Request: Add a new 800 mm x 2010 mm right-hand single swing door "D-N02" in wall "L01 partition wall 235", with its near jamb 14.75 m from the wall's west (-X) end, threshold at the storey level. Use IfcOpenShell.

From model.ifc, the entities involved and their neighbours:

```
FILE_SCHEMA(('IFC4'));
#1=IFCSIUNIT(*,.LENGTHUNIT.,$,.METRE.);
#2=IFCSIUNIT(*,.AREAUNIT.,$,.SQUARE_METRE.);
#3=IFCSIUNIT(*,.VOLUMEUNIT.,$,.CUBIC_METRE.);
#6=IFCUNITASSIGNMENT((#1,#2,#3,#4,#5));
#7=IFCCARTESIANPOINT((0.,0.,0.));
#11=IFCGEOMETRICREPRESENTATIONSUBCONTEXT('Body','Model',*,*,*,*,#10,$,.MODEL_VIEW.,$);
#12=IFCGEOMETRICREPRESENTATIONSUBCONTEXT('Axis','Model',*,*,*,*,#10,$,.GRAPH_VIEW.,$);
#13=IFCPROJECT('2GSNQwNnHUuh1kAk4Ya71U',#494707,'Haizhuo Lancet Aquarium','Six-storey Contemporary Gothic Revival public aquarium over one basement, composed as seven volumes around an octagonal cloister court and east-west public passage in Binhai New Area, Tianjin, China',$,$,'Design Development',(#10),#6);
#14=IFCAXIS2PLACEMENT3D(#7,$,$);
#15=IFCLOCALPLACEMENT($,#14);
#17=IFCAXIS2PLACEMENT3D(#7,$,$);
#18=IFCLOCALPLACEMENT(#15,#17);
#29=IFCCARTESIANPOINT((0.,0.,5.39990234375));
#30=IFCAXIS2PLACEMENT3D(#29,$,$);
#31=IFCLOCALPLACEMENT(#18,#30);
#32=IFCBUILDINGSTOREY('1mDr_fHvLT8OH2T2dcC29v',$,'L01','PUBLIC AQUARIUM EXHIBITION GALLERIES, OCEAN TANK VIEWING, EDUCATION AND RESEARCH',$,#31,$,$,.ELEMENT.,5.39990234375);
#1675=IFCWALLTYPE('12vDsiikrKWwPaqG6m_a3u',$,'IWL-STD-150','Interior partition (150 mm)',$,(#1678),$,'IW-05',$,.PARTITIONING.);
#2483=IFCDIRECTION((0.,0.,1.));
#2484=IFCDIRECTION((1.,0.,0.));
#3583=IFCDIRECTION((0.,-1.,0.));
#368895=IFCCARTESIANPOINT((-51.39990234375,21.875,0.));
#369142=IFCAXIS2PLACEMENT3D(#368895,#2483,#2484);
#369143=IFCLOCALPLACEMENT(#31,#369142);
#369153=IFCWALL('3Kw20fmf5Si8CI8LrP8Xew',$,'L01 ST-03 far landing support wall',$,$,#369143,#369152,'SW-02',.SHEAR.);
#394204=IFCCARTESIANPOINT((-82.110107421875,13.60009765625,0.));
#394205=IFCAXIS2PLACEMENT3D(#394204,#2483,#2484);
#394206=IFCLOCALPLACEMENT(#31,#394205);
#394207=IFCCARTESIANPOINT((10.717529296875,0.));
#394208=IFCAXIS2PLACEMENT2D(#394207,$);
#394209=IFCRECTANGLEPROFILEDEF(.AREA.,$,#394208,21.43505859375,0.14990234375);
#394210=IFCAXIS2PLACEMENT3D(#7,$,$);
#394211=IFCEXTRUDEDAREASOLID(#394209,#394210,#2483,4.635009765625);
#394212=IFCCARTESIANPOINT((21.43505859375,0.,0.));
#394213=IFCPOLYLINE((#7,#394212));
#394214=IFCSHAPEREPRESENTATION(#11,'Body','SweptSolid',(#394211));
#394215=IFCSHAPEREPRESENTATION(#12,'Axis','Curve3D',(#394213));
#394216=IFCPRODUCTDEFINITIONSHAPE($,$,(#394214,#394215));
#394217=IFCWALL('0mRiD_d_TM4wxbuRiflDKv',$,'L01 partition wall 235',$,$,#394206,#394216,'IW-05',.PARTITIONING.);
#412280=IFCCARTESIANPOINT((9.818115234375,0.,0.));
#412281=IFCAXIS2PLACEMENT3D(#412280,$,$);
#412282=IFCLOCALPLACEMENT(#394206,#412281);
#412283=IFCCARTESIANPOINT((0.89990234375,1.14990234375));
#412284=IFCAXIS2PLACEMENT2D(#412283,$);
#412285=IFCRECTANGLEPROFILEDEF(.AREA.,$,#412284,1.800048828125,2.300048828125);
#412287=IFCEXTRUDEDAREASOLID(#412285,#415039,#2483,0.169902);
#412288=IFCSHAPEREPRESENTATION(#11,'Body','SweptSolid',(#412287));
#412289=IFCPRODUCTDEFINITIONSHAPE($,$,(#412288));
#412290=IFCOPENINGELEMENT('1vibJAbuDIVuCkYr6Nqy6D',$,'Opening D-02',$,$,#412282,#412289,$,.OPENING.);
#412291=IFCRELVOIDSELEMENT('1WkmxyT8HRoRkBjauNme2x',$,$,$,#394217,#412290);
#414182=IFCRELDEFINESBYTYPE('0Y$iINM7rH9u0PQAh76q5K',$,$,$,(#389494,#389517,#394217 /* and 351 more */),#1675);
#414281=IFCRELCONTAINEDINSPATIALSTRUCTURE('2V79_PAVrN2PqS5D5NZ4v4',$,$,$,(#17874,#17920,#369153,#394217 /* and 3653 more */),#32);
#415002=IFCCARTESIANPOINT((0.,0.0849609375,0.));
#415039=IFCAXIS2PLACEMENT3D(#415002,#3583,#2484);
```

```python
import numpy as np
import ifcopenshell
import ifcopenshell.api.feature
import ifcopenshell.api.geometry
import ifcopenshell.api.root
import ifcopenshell.api.spatial
import ifcopenshell.geom
import ifcopenshell.util.element
import ifcopenshell.util.placement
import ifcopenshell.util.representation
import ifcopenshell.util.shape
import ifcopenshell.util.unit

model = ifcopenshell.open("model.ifc")
unit_scale = ifcopenshell.util.unit.calculate_unit_scale(model)
settings = ifcopenshell.geom.settings()


def volume(element):
    """Net volume in cubic metres, openings subtracted."""
    shape = ifcopenshell.geom.create_shape(settings, element)
    return ifcopenshell.util.shape.get_volume(shape.geometry)


wall = model.by_id(394217)
storey = ifcopenshell.util.element.get_container(wall, ifc_class="IfcBuildingStorey")
context = ifcopenshell.util.representation.get_context(model, "Model", "Body", "MODEL_VIEW")
before = volume(wall)

width, height, from_end, sill = 0.8, 2.01, 14.75, 0.0  # metres

# The wall runs along its own X axis, and the end named is its -X end.
wall_shape = ifcopenshell.geom.create_shape(settings, wall)
x, y, z = ifcopenshell.util.shape.get_vertices(wall_shape.geometry).T
start = x.min() + from_end
face, thickness = float(y.min()), float(y.max() - y.min())
wall_matrix = ifcopenshell.util.placement.get_local_placement(wall.ObjectPlacement)
level = ifcopenshell.util.placement.get_local_placement(storey.ObjectPlacement)[2, 3]


def in_wall(x, y):
    """Placement at x, y metres in the wall's axes, at sill height."""
    matrix = wall_matrix.copy()
    matrix[:, 3] = wall_matrix @ np.array([x / unit_scale, y / unit_scale, 0.0, 1.0])
    matrix[2, 3] = level + sill / unit_scale
    return matrix


# Opening: a box that overshoots both wall faces by 50 mm.
opening = ifcopenshell.api.root.create_entity(model, ifc_class="IfcOpeningElement", predefined_type="OPENING")
box = ifcopenshell.api.geometry.add_wall_representation(
    model, context=context, length=width, height=height, thickness=thickness + 0.1
)
ifcopenshell.api.geometry.assign_representation(model, product=opening, representation=box)
ifcopenshell.api.geometry.edit_object_placement(model, product=opening, matrix=in_wall(start, face - 0.05), is_si=False)
ifcopenshell.api.feature.add_feature(model, feature=opening, element=wall)

door = ifcopenshell.api.root.create_entity(model, ifc_class="IfcDoor", name="D-N02", predefined_type="DOOR")
door.OverallWidth, door.OverallHeight = width / unit_scale, height / unit_scale
door.OperationType = "SINGLE_SWING_RIGHT"
body = ifcopenshell.api.geometry.add_door_representation(
    model,
    context=context,
    overall_width=door.OverallWidth,
    overall_height=door.OverallHeight,
    operation_type="SINGLE_SWING_RIGHT",
    lining_properties={"LiningDepth": thickness / unit_scale, "ThresholdDepth": thickness / unit_scale},
)
ifcopenshell.api.geometry.assign_representation(model, product=door, representation=body)
ifcopenshell.api.spatial.assign_container(model, products=[door], relating_structure=storey)
ifcopenshell.api.feature.add_filling(model, opening=opening, element=door)

# The lining spans the wall, so the door starts at the wall face.
ifcopenshell.api.geometry.edit_object_placement(model, product=door, matrix=in_wall(start, face), is_si=False)

after = volume(wall)

print(f"wall volume {before:.3f} -> {after:.3f} m3")

model.write("model_rev.ifc")
```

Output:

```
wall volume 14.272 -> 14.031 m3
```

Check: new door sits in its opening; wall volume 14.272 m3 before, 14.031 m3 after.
